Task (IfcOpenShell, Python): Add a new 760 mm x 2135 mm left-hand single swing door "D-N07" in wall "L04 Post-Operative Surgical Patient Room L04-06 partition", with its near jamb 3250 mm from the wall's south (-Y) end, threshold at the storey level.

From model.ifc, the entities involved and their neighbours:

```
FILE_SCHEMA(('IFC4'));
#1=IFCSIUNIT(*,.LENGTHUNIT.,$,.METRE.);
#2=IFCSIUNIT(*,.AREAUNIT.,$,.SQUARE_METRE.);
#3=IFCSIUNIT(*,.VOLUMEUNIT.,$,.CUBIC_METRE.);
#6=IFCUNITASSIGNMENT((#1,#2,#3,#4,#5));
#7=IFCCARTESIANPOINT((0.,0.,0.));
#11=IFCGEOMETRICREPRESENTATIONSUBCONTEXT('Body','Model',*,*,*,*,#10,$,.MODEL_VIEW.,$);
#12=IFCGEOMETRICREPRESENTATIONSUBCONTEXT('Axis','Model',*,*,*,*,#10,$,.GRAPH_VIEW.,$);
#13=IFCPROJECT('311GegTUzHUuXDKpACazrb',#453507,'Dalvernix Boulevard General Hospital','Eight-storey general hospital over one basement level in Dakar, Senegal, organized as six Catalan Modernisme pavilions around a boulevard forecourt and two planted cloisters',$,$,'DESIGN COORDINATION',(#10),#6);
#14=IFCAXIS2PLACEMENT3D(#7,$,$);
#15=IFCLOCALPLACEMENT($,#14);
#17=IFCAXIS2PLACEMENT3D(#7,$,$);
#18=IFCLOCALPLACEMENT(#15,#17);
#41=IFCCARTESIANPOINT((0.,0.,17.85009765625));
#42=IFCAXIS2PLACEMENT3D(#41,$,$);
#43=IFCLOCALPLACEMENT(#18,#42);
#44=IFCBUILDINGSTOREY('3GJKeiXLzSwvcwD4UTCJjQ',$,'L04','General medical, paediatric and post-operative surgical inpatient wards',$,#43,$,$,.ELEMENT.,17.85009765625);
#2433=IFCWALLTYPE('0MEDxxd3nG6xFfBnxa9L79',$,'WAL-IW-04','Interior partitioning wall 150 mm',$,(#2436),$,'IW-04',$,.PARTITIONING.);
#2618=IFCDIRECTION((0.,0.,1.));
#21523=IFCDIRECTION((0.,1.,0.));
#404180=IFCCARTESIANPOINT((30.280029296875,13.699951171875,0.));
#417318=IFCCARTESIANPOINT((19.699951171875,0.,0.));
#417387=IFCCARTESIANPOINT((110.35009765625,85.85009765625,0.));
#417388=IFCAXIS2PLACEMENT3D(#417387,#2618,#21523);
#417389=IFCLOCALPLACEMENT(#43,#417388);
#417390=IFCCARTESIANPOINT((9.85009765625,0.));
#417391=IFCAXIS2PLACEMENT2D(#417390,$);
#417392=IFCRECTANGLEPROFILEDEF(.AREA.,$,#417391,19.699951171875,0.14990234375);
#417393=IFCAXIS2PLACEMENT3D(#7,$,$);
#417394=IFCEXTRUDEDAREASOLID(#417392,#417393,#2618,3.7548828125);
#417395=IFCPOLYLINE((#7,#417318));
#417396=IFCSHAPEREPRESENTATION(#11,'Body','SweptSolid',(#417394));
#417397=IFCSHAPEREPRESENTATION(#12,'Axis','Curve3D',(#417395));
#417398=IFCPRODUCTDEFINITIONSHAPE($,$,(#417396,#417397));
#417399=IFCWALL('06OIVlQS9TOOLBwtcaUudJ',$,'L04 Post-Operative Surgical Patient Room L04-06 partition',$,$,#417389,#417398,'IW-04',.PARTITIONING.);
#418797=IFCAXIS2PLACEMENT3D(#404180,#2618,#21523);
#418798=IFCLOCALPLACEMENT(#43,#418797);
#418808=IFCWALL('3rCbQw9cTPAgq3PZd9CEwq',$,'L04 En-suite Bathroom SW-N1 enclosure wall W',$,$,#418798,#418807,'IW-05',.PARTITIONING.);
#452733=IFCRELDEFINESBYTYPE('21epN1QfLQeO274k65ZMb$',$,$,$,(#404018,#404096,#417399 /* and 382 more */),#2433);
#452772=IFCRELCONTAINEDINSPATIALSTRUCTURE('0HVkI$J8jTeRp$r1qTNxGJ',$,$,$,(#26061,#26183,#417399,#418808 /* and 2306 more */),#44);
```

```python
import numpy as np
import ifcopenshell
import ifcopenshell.api.feature
import ifcopenshell.api.geometry
import ifcopenshell.api.root
import ifcopenshell.api.spatial
import ifcopenshell.geom
import ifcopenshell.util.element
import ifcopenshell.util.placement
import ifcopenshell.util.representation
import ifcopenshell.util.shape
import ifcopenshell.util.unit

model = ifcopenshell.open("model.ifc")
unit_scale = ifcopenshell.util.unit.calculate_unit_scale(model)
settings = ifcopenshell.geom.settings()


def volume(element):
    """Net volume in cubic metres, openings subtracted."""
    shape = ifcopenshell.geom.create_shape(settings, element)
    return ifcopenshell.util.shape.get_volume(shape.geometry)


wall = model.by_guid("06OIVlQS9TOOLBwtcaUudJ")
storey = ifcopenshell.util.element.get_container(wall, ifc_class="IfcBuildingStorey")
context = ifcopenshell.util.representation.get_context(model, "Model", "Body", "MODEL_VIEW")
before = volume(wall)

width, height, from_end, sill = 0.76, 2.135, 3.25, 0.0  # metres

# The wall runs along its own X axis, and the end named is its -X end.
wall_shape = ifcopenshell.geom.create_shape(settings, wall)
x, y, z = ifcopenshell.util.shape.get_vertices(wall_shape.geometry).T
start = x.min() + from_end
face, thickness = float(y.min()), float(y.max() - y.min())
wall_matrix = ifcopenshell.util.placement.get_local_placement(wall.ObjectPlacement)
level = ifcopenshell.util.placement.get_local_placement(storey.ObjectPlacement)[2, 3]


def in_wall(x, y):
    """Placement at x, y metres in the wall's axes, at sill height."""
    matrix = wall_matrix.copy()
    matrix[:, 3] = wall_matrix @ np.array([x / unit_scale, y / unit_scale, 0.0, 1.0])
    matrix[2, 3] = level + sill / unit_scale
    return matrix


# Opening: a box that overshoots both wall faces by 50 mm.
opening = ifcopenshell.api.root.create_entity(model, ifc_class="IfcOpeningElement", predefined_type="OPENING")
box = ifcopenshell.api.geometry.add_wall_representation(
    model, context=context, length=width, height=height, thickness=thickness + 0.1
)
ifcopenshell.api.geometry.assign_representation(model, product=opening, representation=box)
ifcopenshell.api.geometry.edit_object_placement(model, product=opening, matrix=in_wall(start, face - 0.05), is_si=False)
ifcopenshell.api.feature.add_feature(model, feature=opening, element=wall)

door = ifcopenshell.api.root.create_entity(model, ifc_class="IfcDoor", name="D-N07", predefined_type="DOOR")
door.OverallWidth, door.OverallHeight = width / unit_scale, height / unit_scale
door.OperationType = "SINGLE_SWING_LEFT"
body = ifcopenshell.api.geometry.add_door_representation(
    model,
    context=context,
    overall_width=door.OverallWidth,
    overall_height=door.OverallHeight,
    operation_type="SINGLE_SWING_LEFT",
    lining_properties={"LiningDepth": thickness / unit_scale, "ThresholdDepth": thickness / unit_scale},
)
ifcopenshell.api.geometry.assign_representation(model, product=door, representation=body)
ifcopenshell.api.spatial.assign_container(model, products=[door], relating_structure=storey)
ifcopenshell.api.feature.add_filling(model, opening=opening, element=door)

# The lining spans the wall, so the door starts at the wall face.
ifcopenshell.api.geometry.edit_object_placement(model, product=door, matrix=in_wall(start, face), is_si=False)

after = volume(wall)

print(f"wall volume {before:.3f} -> {after:.3f} m3")

model.write("model_rev.ifc")
```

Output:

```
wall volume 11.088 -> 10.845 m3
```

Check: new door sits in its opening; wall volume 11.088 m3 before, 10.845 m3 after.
